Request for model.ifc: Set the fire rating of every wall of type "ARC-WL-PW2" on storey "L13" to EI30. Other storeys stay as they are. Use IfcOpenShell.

First a look at what the model holds.

```python
import ifcopenshell
import ifcopenshell.util.element

model = ifcopenshell.open("model.ifc")
print(model.schema)
storey = next(s for s in model.by_type("IfcBuildingStorey") if s.Name == "L13")
walls = [e for e in ifcopenshell.util.element.get_decomposition(storey) if e.is_a("IfcWall")]
seen = {}
for e in walls:
    element_type = ifcopenshell.util.element.get_type(e)
    key = (element_type.Name if element_type != e and element_type else None, ifcopenshell.util.element.get_pset(e, "Pset_WallCommon", "FireRating"))
    seen[key] = seen.get(key, 0) + 1
for (name, value), count in sorted(seen.items(), key=str):
    print(count, "x", name, "|", value)
```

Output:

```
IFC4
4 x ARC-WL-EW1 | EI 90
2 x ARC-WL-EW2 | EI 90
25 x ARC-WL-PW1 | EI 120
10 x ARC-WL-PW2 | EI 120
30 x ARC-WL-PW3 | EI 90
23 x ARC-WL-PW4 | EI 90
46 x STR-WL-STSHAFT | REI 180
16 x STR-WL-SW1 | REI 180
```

```python
import ifcopenshell
import ifcopenshell.api.pset
import ifcopenshell.util.element

model = ifcopenshell.open("model.ifc")

storey = next(s for s in model.by_type("IfcBuildingStorey") if s.Name == "L13")
walls = [e for e in ifcopenshell.util.element.get_decomposition(storey) if e.is_a("IfcWall")]

count = 0
for e in walls:
    element_type = ifcopenshell.util.element.get_type(e)
    if element_type in (None, e) or element_type.Name != "ARC-WL-PW2":
        continue
    found = ifcopenshell.util.element.get_pset(e, "Pset_WallCommon", should_inherit=False)
    if found:
        pset = model.by_id(found["id"])
        if len(ifcopenshell.util.element.get_elements_by_pset(pset)) > 1:
            pset = ifcopenshell.api.pset.unshare_pset(model, products=[e], pset=pset)[0]
    else:
        pset = ifcopenshell.api.pset.add_pset(model, product=e, name="Pset_WallCommon")
    ifcopenshell.api.pset.edit_pset(model, pset=pset, properties={"FireRating": "EI30"})
    count += 1

print(count, "walls updated")

model.write("model_v2.ifc")
```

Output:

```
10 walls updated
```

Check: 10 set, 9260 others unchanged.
